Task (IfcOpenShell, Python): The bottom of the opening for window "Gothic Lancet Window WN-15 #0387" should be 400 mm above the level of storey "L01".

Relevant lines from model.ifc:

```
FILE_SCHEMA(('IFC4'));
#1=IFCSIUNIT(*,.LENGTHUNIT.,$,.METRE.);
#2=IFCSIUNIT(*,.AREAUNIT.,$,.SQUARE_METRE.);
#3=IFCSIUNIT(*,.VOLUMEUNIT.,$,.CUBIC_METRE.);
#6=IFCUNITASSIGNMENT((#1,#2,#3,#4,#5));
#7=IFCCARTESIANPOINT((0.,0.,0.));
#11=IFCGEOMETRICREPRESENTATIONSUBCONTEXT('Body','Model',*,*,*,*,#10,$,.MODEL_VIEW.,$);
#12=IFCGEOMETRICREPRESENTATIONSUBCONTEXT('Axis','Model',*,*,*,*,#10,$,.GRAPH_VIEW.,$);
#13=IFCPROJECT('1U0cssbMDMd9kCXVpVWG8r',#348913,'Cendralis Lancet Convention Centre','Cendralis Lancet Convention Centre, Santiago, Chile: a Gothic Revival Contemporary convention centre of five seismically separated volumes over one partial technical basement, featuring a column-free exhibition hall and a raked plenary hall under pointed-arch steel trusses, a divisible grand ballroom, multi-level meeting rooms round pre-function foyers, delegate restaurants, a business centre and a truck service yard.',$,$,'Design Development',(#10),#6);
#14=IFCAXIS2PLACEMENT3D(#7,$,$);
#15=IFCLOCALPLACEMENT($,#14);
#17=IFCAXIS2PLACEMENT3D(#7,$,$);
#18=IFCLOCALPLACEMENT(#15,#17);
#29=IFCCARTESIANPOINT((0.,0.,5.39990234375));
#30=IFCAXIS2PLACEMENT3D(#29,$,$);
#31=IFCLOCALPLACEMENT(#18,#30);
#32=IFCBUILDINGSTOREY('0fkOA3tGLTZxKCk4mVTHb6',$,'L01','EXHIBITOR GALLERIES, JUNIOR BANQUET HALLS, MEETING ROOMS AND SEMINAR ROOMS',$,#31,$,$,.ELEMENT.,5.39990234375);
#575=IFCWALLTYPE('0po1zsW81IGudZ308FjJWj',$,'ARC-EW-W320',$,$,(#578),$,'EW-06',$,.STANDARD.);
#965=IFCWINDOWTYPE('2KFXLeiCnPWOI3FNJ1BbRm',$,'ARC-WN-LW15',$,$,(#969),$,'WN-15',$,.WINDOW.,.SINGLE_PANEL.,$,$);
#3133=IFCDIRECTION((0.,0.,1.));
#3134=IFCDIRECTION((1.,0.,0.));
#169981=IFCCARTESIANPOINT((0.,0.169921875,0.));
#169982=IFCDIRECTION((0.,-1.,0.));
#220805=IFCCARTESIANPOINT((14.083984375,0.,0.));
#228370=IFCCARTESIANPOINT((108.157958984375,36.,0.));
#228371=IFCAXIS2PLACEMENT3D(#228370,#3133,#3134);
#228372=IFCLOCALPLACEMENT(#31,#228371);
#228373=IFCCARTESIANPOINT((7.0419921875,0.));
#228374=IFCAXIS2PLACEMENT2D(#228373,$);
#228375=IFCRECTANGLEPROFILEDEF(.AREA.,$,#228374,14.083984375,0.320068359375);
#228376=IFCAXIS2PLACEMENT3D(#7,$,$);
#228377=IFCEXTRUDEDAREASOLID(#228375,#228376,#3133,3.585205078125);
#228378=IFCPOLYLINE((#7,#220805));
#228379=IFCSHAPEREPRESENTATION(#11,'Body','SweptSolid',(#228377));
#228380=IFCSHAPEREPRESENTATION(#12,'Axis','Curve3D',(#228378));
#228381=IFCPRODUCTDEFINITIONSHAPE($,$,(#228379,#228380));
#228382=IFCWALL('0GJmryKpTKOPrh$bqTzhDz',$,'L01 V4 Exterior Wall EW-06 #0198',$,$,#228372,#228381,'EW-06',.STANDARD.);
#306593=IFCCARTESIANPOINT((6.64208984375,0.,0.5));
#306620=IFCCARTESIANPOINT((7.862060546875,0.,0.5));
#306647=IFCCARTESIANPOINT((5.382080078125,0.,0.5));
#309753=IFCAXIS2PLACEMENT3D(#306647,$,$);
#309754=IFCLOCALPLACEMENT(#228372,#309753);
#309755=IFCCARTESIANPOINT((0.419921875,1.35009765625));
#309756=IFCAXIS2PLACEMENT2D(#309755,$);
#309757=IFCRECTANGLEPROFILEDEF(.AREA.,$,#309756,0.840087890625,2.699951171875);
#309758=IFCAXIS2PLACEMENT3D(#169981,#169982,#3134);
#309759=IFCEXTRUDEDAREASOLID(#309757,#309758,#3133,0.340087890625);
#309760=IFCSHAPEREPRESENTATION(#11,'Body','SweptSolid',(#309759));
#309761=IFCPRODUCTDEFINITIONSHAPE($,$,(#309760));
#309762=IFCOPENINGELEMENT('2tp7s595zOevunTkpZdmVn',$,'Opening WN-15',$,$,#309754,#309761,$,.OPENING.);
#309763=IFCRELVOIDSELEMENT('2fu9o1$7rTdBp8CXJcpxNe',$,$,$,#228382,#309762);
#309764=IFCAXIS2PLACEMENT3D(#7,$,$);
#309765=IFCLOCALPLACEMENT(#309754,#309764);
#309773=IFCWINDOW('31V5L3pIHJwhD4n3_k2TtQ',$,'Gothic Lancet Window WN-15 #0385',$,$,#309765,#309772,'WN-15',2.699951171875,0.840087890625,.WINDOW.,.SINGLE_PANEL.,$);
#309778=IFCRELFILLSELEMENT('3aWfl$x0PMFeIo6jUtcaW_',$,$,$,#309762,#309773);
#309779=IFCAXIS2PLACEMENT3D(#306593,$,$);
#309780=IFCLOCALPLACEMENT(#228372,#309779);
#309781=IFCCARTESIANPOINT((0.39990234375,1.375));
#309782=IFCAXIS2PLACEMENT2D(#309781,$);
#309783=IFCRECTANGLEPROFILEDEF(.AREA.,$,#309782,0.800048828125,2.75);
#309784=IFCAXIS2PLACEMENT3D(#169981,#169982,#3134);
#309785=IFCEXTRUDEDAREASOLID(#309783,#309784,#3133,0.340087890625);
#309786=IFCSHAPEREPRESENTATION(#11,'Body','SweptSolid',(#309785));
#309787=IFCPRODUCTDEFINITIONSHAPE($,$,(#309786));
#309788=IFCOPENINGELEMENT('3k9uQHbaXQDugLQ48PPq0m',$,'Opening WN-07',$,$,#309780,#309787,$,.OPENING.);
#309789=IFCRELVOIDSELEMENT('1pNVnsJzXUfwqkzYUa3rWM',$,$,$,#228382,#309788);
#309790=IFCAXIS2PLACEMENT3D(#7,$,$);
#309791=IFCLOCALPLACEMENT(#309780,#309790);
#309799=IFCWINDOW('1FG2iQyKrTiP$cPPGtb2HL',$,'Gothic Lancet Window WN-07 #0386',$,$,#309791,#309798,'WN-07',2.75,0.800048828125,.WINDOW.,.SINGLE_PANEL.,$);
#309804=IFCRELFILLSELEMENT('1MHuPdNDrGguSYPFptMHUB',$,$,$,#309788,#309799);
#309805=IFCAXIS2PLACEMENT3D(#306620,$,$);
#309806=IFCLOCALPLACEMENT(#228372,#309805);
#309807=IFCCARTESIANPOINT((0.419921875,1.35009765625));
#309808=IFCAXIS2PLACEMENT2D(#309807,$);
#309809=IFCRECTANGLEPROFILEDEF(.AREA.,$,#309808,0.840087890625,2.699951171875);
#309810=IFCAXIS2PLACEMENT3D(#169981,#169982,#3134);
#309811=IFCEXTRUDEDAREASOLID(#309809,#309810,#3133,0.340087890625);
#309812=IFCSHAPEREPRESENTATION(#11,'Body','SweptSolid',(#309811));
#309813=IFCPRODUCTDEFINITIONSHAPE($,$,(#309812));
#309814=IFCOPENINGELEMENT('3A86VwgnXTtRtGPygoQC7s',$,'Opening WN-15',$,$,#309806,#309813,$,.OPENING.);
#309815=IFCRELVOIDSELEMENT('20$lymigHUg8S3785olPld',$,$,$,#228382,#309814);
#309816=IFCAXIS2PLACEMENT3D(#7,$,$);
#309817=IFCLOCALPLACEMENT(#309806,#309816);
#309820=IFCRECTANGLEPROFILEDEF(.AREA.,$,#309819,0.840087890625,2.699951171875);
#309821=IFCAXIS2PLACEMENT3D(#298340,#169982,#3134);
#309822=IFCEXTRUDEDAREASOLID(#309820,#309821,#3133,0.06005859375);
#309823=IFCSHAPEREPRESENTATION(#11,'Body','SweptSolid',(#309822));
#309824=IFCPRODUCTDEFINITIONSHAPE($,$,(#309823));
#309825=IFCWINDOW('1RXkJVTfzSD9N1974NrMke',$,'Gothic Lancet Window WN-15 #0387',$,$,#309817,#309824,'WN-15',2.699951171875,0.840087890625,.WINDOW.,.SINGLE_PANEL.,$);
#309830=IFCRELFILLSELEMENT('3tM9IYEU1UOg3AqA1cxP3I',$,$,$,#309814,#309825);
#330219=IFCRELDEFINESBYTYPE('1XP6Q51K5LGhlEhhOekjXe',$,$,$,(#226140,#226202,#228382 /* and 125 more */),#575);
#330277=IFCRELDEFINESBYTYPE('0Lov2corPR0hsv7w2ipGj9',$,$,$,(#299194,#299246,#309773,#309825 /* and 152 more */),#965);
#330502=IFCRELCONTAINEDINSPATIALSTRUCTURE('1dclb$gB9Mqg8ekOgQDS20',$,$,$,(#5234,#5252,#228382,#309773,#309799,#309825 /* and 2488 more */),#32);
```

```python
import numpy as np
import ifcopenshell
import ifcopenshell.api.geometry
import ifcopenshell.geom
import ifcopenshell.util.element
import ifcopenshell.util.placement
import ifcopenshell.util.shape
import ifcopenshell.util.unit

model = ifcopenshell.open("model.ifc")
unit_scale = ifcopenshell.util.unit.calculate_unit_scale(model)

window = model.by_id(309825)
opening = window.FillsVoids[0].RelatingOpeningElement
storey = ifcopenshell.util.element.get_container(window, ifc_class="IfcBuildingStorey")
level = ifcopenshell.util.placement.get_local_placement(storey.ObjectPlacement)[2, 3]

# The opening's origin need not be at the sill, so measure its lowest point.
shape = ifcopenshell.geom.create_shape(ifcopenshell.geom.settings(), opening)
bottom = ifcopenshell.util.shape.get_shape_bottom_elevation(shape, shape.geometry) / unit_scale
dz = level + 0.4 - bottom

shift = np.array([0.0, 0.0, dz])
# The window is placed relative to its opening, so it follows when the opening moves.
matrix = ifcopenshell.util.placement.get_local_placement(opening.ObjectPlacement)
matrix[:3, 3] += shift
ifcopenshell.api.geometry.edit_object_placement(
    model, product=opening, matrix=matrix, is_si=False, should_transform_children=True
)

print(f"moved by {dz * unit_scale:+.3f} m")

model.write("model-out.ifc")
```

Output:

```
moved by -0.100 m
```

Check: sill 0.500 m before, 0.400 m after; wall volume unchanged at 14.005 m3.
